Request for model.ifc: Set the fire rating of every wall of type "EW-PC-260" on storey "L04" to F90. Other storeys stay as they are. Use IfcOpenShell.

First a look at what the model holds.

```python
import ifcopenshell
import ifcopenshell.util.element

model = ifcopenshell.open("model.ifc")
print(model.schema)
storey = next(s for s in model.by_type("IfcBuildingStorey") if s.Name == "L04")
walls = [e for e in ifcopenshell.util.element.get_decomposition(storey) if e.is_a("IfcWall")]
seen = {}
for e in walls:
    element_type = ifcopenshell.util.element.get_type(e)
    key = (element_type.Name if element_type != e and element_type else None, ifcopenshell.util.element.get_pset(e, "Pset_WallCommon", "FireRating"))
    seen[key] = seen.get(key, 0) + 1
for (name, value), count in sorted(seen.items(), key=str):
    print(count, "x", name, "|", value)
```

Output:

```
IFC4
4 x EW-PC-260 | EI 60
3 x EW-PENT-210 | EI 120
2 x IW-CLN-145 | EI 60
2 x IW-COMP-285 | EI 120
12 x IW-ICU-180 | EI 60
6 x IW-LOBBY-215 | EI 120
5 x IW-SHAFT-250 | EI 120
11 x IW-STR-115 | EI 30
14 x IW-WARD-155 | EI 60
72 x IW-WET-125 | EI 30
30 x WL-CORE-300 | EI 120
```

```python
import ifcopenshell
import ifcopenshell.api.pset
import ifcopenshell.util.element

model = ifcopenshell.open("model.ifc")

storey = next(s for s in model.by_type("IfcBuildingStorey") if s.Name == "L04")
walls = [e for e in ifcopenshell.util.element.get_decomposition(storey) if e.is_a("IfcWall")]

count = 0
for e in walls:
    element_type = ifcopenshell.util.element.get_type(e)
    if element_type in (None, e) or element_type.Name != "EW-PC-260":
        continue
    # add_pset returns the element's existing set when there is one.
    pset = ifcopenshell.api.pset.add_pset(model, product=e, name="Pset_WallCommon")
    ifcopenshell.api.pset.edit_pset(model, pset=pset, properties={"FireRating": "F90"})
    count += 1

print(count, "walls updated")

model.write("model-out.ifc")
```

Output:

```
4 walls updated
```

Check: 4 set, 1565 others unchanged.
